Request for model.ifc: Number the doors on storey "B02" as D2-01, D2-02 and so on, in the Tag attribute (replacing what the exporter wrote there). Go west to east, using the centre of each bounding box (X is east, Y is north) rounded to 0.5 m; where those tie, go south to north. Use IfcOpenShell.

First a look at what the model holds.

```python
import ifcopenshell
import ifcopenshell.util.element
import ifcopenshell.util.placement

model = ifcopenshell.open("model.ifc")
print(model.schema)
storey = next(s for s in model.by_type("IfcBuildingStorey") if s.Name == "B02")
doors = [e for e in ifcopenshell.util.element.get_decomposition(storey) if e.is_a("IfcDoor")]
for e in sorted(doors, key=lambda e: e.id()):
    origin = ifcopenshell.util.placement.get_local_placement(e.ObjectPlacement)[:3, 3]
    print(e.id(), e.Tag, e.Name, origin.round(2) + 0.0, sep=" | ")
```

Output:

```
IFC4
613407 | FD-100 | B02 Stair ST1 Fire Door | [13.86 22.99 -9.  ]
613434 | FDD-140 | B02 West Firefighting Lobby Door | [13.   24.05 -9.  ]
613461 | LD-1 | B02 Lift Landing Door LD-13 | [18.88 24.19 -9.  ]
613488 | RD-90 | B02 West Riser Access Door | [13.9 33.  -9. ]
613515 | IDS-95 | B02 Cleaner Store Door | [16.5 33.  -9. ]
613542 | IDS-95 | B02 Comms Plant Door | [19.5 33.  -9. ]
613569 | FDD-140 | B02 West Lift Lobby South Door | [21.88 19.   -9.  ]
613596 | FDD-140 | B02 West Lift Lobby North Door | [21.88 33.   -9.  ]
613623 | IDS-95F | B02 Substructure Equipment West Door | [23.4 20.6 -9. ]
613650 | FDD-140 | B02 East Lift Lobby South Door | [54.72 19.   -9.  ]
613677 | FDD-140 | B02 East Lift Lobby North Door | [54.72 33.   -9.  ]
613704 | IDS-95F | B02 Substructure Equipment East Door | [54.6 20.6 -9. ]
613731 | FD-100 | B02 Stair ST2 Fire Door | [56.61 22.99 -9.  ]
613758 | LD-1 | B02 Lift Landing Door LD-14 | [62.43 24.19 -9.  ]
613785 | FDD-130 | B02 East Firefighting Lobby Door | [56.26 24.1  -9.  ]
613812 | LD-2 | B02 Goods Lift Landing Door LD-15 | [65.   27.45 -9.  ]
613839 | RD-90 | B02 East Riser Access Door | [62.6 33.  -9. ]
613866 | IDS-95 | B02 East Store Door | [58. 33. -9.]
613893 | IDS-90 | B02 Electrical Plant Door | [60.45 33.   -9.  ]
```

```python
import ifcopenshell
import ifcopenshell.geom
import ifcopenshell.util.element
import ifcopenshell.util.shape

model = ifcopenshell.open("model.ifc")
settings = ifcopenshell.geom.settings()
settings.set("use-world-coords", True)


def centre(element):
    shape = ifcopenshell.geom.create_shape(settings, element)
    return ifcopenshell.util.shape.get_bbox_centroid(shape.geometry)


storey = next(s for s in model.by_type("IfcBuildingStorey") if s.Name == "B02")
doors = [e for e in ifcopenshell.util.element.get_decomposition(storey) if e.is_a("IfcDoor")]

# Insertion points can sit at a corner or the storey origin, so sort by the geometry (in metres).
centres = {e: centre(e) for e in doors}
doors.sort(key=lambda e: (round(centres[e][0] / 0.5), centres[e][1]))

for i, e in enumerate(doors, start=1):
    number = f"D2-{i:02d}"
    e.Tag = number
    print(e.id(), number)

model.write("model_v2.ifc")
```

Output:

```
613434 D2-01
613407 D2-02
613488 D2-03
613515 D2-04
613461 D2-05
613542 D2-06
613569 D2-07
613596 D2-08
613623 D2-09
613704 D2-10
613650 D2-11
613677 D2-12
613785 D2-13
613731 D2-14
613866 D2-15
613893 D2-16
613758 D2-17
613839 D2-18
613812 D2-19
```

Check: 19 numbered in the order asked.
